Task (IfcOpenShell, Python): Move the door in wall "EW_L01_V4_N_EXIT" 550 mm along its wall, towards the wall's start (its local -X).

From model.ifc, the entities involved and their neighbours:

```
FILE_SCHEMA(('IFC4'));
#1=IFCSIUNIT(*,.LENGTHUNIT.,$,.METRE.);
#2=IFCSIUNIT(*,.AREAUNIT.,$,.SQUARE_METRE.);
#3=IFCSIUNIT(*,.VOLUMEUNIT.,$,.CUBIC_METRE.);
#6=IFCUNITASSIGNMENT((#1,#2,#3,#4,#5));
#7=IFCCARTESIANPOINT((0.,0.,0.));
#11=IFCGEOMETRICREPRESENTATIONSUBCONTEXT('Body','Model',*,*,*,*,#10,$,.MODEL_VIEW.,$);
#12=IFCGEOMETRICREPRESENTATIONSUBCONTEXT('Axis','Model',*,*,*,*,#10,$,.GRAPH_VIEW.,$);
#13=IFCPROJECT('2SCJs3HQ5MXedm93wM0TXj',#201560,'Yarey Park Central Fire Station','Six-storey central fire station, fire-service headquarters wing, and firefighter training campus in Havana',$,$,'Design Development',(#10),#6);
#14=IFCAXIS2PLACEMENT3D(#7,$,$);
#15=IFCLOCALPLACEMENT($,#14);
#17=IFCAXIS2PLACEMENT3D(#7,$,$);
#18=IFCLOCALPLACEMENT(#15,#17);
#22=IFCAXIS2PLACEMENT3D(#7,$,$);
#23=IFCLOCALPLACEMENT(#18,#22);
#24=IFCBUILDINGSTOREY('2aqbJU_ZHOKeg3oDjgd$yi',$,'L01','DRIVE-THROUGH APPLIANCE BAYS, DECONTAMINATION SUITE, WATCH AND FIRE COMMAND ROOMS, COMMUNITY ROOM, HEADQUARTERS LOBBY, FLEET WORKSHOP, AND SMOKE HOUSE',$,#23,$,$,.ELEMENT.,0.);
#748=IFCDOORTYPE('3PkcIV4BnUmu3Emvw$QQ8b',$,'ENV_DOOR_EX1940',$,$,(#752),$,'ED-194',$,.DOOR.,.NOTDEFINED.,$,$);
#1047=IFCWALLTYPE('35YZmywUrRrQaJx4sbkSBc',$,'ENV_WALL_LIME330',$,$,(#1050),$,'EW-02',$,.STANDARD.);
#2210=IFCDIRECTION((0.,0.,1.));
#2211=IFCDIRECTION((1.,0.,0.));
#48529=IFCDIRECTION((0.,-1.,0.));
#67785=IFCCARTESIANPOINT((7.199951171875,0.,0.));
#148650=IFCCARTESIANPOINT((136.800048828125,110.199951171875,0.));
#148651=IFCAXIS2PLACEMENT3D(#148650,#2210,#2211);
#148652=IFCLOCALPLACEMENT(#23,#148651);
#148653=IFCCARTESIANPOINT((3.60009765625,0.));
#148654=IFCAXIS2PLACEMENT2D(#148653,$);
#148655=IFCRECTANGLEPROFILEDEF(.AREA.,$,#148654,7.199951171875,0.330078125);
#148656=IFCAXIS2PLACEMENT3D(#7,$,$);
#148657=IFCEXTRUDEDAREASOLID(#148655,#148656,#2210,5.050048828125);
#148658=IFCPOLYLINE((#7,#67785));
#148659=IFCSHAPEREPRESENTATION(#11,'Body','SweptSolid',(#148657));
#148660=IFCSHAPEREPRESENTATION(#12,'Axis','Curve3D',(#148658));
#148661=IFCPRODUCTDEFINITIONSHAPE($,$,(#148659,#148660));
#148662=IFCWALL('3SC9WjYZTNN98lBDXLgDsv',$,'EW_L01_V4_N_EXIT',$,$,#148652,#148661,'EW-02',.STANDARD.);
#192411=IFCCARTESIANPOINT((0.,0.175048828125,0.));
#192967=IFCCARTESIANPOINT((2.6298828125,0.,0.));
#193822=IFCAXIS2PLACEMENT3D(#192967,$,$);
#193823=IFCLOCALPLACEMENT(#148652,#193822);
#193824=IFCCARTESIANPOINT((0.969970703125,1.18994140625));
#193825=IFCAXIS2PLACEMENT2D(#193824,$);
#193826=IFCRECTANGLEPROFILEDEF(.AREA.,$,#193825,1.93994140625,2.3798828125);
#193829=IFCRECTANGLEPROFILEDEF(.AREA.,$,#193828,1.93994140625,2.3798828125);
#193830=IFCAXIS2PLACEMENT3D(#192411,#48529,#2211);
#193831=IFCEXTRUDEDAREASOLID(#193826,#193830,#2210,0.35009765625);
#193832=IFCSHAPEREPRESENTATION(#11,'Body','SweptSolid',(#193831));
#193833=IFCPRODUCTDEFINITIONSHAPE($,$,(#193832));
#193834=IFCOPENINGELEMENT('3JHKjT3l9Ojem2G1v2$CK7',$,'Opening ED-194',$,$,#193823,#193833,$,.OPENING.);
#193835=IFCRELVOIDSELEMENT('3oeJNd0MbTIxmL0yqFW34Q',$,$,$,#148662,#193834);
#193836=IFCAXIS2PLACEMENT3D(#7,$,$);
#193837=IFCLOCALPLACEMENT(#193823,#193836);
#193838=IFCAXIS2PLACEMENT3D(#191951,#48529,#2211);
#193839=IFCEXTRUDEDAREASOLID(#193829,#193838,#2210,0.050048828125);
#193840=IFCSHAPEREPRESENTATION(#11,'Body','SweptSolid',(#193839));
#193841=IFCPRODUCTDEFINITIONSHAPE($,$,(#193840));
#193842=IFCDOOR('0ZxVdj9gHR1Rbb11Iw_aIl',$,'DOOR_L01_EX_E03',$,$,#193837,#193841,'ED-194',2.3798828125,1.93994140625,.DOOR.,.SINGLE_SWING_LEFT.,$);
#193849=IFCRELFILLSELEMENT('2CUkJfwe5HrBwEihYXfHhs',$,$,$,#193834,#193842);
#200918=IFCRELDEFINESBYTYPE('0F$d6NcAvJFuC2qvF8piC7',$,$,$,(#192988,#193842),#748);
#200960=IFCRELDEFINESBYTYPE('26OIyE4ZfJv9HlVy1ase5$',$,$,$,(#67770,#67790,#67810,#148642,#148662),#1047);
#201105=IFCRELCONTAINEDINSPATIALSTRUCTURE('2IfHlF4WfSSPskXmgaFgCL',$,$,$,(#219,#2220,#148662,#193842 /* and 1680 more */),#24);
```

```python
import ifcopenshell
import ifcopenshell.api.geometry
import ifcopenshell.util.placement
import ifcopenshell.util.unit

model = ifcopenshell.open("model.ifc")
unit_scale = ifcopenshell.util.unit.calculate_unit_scale(model)

door = model.by_guid("0ZxVdj9gHR1Rbb11Iw_aIl")
opening = door.FillsVoids[0].RelatingOpeningElement
wall = opening.VoidsElements[0].RelatingBuildingElement

wall_matrix = ifcopenshell.util.placement.get_local_placement(wall.ObjectPlacement)
shift = wall_matrix[:3, 0] * -0.55 / unit_scale
before = ifcopenshell.util.placement.get_local_placement(door.ObjectPlacement)[:3, 3].copy()

# The door is placed relative to its opening, so it follows when the opening moves.
matrix = ifcopenshell.util.placement.get_local_placement(opening.ObjectPlacement)
matrix[:3, 3] += shift
ifcopenshell.api.geometry.edit_object_placement(
    model, product=opening, matrix=matrix, is_si=False, should_transform_children=True
)

after = ifcopenshell.util.placement.get_local_placement(door.ObjectPlacement)[:3, 3]
print("door moved by", (after - before).round(3) + 0.0)

model.write("model_updated.ifc")
```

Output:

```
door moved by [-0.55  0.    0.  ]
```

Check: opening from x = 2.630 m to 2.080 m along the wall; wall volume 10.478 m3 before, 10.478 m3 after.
